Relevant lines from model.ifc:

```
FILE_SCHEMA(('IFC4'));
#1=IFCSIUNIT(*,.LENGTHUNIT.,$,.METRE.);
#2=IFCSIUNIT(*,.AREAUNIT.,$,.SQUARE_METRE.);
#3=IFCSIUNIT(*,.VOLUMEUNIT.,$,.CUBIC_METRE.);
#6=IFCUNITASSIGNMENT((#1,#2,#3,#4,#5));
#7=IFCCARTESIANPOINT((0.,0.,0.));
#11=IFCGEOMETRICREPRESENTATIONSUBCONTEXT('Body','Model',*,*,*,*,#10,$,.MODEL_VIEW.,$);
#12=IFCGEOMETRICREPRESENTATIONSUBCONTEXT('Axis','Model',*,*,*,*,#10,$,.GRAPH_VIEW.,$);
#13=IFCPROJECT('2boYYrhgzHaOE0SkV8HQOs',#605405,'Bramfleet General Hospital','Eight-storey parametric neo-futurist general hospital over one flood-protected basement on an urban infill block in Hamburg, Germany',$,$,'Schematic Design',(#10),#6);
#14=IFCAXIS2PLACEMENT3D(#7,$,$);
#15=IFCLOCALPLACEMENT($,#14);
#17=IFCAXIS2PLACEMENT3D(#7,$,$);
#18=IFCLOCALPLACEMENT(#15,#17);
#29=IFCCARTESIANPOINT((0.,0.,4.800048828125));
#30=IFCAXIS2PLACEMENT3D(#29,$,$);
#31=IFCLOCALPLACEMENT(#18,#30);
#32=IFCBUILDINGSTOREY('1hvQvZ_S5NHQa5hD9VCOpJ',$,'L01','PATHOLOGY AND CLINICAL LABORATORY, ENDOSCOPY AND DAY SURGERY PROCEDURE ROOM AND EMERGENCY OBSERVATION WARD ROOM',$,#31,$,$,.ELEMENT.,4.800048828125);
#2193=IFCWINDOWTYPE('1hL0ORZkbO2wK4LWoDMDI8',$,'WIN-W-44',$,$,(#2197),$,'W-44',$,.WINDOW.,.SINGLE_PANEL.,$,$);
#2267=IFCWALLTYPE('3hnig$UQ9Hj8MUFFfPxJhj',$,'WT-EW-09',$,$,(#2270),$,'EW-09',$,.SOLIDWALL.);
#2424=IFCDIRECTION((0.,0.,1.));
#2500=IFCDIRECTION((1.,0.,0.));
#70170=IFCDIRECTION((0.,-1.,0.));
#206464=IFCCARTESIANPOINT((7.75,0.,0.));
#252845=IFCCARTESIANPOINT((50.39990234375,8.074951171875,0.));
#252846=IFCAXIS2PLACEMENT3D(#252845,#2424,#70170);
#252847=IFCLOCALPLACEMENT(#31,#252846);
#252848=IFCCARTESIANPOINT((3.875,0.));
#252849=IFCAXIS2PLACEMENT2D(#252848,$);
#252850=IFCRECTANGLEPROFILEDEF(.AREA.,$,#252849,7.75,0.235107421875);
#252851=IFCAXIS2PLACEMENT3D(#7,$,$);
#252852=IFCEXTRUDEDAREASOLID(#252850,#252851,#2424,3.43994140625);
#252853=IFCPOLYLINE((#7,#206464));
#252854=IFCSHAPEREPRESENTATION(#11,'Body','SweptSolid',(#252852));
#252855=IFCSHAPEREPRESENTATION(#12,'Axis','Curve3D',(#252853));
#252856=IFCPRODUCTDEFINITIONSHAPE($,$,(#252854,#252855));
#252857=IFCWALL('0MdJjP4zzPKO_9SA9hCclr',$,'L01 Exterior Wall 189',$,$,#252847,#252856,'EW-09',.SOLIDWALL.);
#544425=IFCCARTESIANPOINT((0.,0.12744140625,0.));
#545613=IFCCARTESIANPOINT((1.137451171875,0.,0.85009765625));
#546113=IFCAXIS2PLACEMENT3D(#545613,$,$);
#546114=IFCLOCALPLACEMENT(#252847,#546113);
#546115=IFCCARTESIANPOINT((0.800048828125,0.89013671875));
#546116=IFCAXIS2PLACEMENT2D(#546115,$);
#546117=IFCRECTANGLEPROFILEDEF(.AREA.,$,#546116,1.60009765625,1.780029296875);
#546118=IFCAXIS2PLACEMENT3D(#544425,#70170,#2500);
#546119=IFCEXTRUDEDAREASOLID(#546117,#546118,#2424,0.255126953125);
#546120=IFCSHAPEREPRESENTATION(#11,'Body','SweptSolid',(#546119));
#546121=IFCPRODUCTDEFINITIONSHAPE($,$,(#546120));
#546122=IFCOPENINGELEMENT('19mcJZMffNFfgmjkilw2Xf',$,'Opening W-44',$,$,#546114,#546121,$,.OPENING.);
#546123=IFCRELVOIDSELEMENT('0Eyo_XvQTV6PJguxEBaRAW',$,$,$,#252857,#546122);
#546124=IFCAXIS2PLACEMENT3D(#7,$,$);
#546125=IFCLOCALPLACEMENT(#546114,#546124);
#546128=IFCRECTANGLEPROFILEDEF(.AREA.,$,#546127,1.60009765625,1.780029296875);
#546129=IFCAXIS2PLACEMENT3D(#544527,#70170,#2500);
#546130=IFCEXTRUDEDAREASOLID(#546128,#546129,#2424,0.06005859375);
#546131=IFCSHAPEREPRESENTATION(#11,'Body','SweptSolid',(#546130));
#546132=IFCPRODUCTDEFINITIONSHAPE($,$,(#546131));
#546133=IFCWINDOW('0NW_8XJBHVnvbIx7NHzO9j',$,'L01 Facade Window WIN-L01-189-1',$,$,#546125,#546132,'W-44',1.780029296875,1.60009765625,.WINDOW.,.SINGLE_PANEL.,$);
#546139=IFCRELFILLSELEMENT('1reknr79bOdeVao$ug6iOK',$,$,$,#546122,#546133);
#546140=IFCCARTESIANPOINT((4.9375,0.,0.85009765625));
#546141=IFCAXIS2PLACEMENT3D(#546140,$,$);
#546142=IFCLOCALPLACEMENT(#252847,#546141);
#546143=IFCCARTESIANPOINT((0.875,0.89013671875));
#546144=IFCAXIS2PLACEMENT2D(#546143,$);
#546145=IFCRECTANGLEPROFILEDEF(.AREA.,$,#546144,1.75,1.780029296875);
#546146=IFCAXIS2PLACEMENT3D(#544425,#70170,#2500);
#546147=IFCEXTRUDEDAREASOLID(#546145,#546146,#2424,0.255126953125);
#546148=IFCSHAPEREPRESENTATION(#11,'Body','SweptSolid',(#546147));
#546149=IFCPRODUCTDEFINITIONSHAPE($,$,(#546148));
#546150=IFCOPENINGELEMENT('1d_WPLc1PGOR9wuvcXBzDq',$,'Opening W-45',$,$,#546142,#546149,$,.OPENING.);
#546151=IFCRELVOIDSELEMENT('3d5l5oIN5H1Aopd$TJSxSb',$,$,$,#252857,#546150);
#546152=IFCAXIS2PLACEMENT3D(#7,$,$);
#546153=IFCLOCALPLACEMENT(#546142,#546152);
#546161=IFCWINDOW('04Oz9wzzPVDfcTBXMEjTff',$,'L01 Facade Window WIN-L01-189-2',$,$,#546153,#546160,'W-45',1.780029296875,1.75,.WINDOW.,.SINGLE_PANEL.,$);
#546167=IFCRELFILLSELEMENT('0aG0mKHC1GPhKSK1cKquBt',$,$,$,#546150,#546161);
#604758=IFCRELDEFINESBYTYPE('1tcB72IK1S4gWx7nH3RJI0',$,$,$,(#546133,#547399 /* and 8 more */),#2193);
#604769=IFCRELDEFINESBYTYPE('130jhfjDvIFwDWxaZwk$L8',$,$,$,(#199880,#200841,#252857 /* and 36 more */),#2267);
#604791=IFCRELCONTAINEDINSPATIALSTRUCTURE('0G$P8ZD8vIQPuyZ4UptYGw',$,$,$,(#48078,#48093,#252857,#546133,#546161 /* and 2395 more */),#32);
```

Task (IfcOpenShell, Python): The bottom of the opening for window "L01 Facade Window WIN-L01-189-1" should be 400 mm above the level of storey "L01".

```python
import numpy as np
import ifcopenshell
import ifcopenshell.api.geometry
import ifcopenshell.geom
import ifcopenshell.util.element
import ifcopenshell.util.placement
import ifcopenshell.util.shape
import ifcopenshell.util.unit

model = ifcopenshell.open("model.ifc")
unit_scale = ifcopenshell.util.unit.calculate_unit_scale(model)

window = model.by_guid("0NW_8XJBHVnvbIx7NHzO9j")
opening = window.FillsVoids[0].RelatingOpeningElement
storey = ifcopenshell.util.element.get_container(window, ifc_class="IfcBuildingStorey")
level = ifcopenshell.util.placement.get_local_placement(storey.ObjectPlacement)[2, 3]

# The opening's origin need not be at the sill, so measure its lowest point.
shape = ifcopenshell.geom.create_shape(ifcopenshell.geom.settings(), opening)
bottom = ifcopenshell.util.shape.get_shape_bottom_elevation(shape, shape.geometry) / unit_scale
dz = level + 0.4 - bottom

shift = np.array([0.0, 0.0, dz])
# The window is placed relative to its opening, so it follows when the opening moves.
matrix = ifcopenshell.util.placement.get_local_placement(opening.ObjectPlacement)
matrix[:3, 3] += shift
ifcopenshell.api.geometry.edit_object_placement(
    model, product=opening, matrix=matrix, is_si=False, should_transform_children=True
)

print(f"moved by {dz * unit_scale:+.3f} m")

model.write("model_v2.ifc")
```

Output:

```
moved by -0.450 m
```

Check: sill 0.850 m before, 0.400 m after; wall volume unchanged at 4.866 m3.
